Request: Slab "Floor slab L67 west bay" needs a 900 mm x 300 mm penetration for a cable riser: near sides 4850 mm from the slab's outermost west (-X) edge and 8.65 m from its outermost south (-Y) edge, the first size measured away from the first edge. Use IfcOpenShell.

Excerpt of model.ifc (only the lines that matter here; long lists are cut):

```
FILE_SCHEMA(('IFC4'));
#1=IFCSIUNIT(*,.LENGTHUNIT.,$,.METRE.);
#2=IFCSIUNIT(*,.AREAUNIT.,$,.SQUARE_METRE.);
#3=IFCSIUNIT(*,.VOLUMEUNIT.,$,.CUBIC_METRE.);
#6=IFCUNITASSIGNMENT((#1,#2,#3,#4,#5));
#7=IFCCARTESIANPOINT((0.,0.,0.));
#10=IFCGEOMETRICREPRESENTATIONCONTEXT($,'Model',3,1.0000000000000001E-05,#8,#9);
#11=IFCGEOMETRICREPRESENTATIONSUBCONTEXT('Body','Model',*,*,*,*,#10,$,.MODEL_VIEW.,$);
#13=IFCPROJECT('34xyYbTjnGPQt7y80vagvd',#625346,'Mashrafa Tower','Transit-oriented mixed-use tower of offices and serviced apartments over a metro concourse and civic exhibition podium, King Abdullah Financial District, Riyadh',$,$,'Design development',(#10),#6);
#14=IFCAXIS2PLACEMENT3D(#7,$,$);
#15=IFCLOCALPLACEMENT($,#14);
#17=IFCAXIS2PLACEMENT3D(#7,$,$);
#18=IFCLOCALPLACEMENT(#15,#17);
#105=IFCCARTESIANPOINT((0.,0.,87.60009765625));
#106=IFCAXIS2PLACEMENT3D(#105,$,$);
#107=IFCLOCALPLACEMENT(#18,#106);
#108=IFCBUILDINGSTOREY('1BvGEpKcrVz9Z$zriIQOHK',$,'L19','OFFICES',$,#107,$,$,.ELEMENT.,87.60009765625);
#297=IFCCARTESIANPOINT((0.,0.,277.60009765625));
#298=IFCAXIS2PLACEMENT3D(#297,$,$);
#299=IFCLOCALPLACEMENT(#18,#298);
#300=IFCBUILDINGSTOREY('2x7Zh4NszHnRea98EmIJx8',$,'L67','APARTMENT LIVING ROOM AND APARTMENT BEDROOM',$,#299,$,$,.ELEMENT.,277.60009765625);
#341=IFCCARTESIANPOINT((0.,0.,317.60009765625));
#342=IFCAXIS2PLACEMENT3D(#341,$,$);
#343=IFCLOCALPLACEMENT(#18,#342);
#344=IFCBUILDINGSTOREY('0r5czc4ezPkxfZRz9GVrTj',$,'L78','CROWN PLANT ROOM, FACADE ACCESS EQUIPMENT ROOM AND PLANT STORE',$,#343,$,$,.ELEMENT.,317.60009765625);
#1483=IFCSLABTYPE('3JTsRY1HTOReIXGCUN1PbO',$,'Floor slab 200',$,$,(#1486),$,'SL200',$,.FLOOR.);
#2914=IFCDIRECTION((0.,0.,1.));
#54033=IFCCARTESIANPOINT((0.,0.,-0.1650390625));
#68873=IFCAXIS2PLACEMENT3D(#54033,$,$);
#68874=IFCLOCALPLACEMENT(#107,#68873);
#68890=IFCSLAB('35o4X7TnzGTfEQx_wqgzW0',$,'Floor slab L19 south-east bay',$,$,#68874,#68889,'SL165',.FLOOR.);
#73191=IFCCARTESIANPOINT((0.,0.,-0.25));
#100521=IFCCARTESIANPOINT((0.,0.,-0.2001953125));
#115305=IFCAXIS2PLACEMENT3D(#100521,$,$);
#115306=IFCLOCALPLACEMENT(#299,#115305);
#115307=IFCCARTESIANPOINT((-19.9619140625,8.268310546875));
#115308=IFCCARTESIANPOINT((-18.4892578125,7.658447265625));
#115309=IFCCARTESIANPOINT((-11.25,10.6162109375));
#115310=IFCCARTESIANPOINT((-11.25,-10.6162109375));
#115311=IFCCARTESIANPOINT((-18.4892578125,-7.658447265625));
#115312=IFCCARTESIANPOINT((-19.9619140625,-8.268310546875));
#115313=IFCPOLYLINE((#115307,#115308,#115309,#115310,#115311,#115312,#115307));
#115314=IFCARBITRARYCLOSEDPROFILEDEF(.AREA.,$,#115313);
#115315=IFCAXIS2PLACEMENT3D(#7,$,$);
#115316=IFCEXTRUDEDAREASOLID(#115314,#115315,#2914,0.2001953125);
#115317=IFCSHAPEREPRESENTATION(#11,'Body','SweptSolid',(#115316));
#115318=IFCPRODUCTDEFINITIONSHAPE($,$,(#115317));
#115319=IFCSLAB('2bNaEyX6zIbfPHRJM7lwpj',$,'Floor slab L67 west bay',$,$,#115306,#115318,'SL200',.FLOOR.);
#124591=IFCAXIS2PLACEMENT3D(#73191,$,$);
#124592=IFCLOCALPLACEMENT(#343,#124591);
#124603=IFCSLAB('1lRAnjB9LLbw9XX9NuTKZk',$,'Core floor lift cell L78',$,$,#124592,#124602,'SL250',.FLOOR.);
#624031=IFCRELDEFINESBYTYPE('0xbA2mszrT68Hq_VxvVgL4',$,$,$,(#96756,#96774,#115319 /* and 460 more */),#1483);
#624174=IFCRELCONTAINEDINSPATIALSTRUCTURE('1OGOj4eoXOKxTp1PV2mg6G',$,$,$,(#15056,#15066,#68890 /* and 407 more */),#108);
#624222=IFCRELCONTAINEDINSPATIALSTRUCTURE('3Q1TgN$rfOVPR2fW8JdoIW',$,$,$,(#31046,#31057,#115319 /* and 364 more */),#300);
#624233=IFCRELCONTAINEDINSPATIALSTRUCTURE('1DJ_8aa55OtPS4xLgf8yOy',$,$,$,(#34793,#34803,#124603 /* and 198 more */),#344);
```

```python
import numpy as np
import ifcopenshell
import ifcopenshell.api.feature
import ifcopenshell.api.geometry
import ifcopenshell.api.root
import ifcopenshell.geom
import ifcopenshell.util.placement
import ifcopenshell.util.representation
import ifcopenshell.util.shape
import ifcopenshell.util.unit

model = ifcopenshell.open("model.ifc")
unit_scale = ifcopenshell.util.unit.calculate_unit_scale(model)
settings = ifcopenshell.geom.settings()


def volume(element):
    """Net volume in cubic metres, openings subtracted."""
    shape = ifcopenshell.geom.create_shape(settings, element)
    return ifcopenshell.util.shape.get_volume(shape.geometry)


slab = model.by_guid("2bNaEyX6zIbfPHRJM7lwpj")
before = volume(slab)

# Extent in the slab's own axes, in metres. The edges named are its -X and -Y sides.
slab_shape = ifcopenshell.geom.create_shape(settings, slab)
vertices = ifcopenshell.util.shape.get_vertices(slab_shape.geometry)
x_min, y_min, bottom = vertices.min(axis=0)
top = vertices[:, 2].max()

opening = ifcopenshell.api.root.create_entity(model, ifc_class="IfcOpeningElement", name="Cable riser opening", predefined_type="OPENING")
context = ifcopenshell.util.representation.get_context(model, "Model", "Body", "MODEL_VIEW")
width, depth = 0.9, 0.3
outline = [(0.0, 0.0), (width, 0.0), (width, depth), (0.0, depth), (0.0, 0.0)]
# Overshoot both faces by 50 mm so the cut is clean.
shape = ifcopenshell.api.geometry.add_slab_representation(
    model, context=context, depth=top - bottom + 0.1, polyline=outline
)
ifcopenshell.api.geometry.assign_representation(model, product=opening, representation=shape)

matrix = ifcopenshell.util.placement.get_local_placement(slab.ObjectPlacement)
matrix[:, 3] = matrix @ np.append(np.array([x_min + 4.85, y_min + 8.65, bottom - 0.05]) / unit_scale, 1.0)
ifcopenshell.api.geometry.edit_object_placement(model, product=opening, matrix=matrix, is_si=False)
ifcopenshell.api.feature.add_feature(model, feature=opening, element=slab)

after = volume(slab)

print(f"slab volume {before:.3f} -> {after:.3f} m3")

model.write("model_updated.ifc")
```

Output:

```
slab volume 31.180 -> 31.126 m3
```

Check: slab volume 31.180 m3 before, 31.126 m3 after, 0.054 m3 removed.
